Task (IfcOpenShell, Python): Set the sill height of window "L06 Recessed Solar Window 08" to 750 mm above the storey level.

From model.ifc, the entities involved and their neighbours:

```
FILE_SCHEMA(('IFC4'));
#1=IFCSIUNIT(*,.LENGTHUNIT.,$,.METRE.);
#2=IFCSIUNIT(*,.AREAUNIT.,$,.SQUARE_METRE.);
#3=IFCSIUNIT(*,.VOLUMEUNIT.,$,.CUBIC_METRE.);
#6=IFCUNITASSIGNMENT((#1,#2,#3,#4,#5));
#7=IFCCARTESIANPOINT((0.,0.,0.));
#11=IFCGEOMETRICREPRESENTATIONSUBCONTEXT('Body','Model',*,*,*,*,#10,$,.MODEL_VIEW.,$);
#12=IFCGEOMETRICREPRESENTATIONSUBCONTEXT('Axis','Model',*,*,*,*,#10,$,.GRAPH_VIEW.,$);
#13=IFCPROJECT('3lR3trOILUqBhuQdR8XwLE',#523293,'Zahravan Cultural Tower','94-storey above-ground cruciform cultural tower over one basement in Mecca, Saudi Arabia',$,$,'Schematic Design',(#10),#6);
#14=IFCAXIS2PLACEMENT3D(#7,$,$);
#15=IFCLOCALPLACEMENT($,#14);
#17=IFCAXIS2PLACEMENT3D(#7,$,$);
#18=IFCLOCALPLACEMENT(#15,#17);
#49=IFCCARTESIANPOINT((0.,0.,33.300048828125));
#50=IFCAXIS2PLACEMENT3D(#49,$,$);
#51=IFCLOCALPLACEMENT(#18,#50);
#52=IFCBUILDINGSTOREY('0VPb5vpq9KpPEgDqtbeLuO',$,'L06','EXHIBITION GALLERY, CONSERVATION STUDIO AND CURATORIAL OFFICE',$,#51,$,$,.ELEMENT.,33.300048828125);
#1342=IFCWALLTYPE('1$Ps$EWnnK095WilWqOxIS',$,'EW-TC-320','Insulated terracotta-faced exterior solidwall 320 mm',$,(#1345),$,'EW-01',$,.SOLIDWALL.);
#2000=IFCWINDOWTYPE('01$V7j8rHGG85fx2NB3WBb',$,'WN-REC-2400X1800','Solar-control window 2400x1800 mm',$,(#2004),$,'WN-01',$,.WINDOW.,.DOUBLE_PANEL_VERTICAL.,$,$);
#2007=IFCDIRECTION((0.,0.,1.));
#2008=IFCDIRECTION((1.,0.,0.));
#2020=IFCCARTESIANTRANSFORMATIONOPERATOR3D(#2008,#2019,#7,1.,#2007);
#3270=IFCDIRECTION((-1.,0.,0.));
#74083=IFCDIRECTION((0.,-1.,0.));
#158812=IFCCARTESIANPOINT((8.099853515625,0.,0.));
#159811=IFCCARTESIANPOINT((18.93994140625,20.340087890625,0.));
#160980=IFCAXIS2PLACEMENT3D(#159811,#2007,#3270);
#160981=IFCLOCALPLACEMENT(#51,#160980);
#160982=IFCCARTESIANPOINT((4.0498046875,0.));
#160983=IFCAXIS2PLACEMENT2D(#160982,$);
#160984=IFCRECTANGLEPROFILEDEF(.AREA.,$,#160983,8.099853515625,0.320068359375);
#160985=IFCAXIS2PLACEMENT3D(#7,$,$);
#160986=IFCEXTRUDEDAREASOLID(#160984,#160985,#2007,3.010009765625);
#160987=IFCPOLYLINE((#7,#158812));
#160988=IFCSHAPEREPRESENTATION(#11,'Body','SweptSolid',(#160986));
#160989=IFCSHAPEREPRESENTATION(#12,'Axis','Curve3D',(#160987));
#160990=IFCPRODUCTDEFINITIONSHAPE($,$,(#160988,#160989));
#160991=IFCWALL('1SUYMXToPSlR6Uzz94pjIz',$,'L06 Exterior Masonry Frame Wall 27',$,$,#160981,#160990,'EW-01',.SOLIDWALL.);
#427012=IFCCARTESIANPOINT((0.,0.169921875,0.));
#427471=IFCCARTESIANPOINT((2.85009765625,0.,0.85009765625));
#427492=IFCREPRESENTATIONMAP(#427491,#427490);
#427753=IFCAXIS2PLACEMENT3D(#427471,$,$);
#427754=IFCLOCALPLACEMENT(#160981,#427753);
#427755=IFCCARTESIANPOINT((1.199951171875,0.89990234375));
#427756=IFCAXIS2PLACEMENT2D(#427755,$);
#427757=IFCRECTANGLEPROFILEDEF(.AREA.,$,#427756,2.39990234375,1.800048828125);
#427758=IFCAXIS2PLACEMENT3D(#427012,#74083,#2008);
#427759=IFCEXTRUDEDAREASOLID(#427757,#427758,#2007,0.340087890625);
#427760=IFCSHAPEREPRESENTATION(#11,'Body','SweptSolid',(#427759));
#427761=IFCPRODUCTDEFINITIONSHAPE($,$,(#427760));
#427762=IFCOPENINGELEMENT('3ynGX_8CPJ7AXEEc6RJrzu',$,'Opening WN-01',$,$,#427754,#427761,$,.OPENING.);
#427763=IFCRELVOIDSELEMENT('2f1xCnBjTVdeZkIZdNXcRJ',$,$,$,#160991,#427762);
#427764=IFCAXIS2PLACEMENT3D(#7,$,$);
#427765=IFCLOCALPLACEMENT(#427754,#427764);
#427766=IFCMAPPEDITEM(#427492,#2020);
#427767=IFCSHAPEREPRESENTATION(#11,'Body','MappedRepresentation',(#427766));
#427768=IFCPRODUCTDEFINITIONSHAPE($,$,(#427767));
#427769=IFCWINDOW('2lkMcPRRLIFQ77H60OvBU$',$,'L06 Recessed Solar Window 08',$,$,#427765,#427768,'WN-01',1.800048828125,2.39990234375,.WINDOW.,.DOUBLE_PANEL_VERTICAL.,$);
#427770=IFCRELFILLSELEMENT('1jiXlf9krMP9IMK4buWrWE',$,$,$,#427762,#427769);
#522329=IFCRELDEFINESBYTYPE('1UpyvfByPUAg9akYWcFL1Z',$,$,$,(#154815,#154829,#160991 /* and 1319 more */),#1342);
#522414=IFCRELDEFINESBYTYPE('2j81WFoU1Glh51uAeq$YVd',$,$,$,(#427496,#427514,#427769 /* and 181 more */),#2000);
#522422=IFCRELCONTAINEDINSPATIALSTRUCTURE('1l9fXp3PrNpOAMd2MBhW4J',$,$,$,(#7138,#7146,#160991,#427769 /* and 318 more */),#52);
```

```python
import numpy as np
import ifcopenshell
import ifcopenshell.api.geometry
import ifcopenshell.geom
import ifcopenshell.util.element
import ifcopenshell.util.placement
import ifcopenshell.util.shape
import ifcopenshell.util.unit

model = ifcopenshell.open("model.ifc")
unit_scale = ifcopenshell.util.unit.calculate_unit_scale(model)

window = model.by_id(427769)
opening = window.FillsVoids[0].RelatingOpeningElement
storey = ifcopenshell.util.element.get_container(window, ifc_class="IfcBuildingStorey")
level = ifcopenshell.util.placement.get_local_placement(storey.ObjectPlacement)[2, 3]

# The opening's origin need not be at the sill, so measure its lowest point.
shape = ifcopenshell.geom.create_shape(ifcopenshell.geom.settings(), opening)
bottom = ifcopenshell.util.shape.get_shape_bottom_elevation(shape, shape.geometry) / unit_scale
dz = level + 0.75 / unit_scale - bottom

shift = np.array([0.0, 0.0, dz])
# The window is placed relative to its opening, so it follows when the opening moves.
matrix = ifcopenshell.util.placement.get_local_placement(opening.ObjectPlacement)
matrix[:3, 3] += shift
ifcopenshell.api.geometry.edit_object_placement(
    model, product=opening, matrix=matrix, is_si=False, should_transform_children=True
)

print(f"moved by {dz * unit_scale:+.3f} m")

model.write("model_rev.ifc")
```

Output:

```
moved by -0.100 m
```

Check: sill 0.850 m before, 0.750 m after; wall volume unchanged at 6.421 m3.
